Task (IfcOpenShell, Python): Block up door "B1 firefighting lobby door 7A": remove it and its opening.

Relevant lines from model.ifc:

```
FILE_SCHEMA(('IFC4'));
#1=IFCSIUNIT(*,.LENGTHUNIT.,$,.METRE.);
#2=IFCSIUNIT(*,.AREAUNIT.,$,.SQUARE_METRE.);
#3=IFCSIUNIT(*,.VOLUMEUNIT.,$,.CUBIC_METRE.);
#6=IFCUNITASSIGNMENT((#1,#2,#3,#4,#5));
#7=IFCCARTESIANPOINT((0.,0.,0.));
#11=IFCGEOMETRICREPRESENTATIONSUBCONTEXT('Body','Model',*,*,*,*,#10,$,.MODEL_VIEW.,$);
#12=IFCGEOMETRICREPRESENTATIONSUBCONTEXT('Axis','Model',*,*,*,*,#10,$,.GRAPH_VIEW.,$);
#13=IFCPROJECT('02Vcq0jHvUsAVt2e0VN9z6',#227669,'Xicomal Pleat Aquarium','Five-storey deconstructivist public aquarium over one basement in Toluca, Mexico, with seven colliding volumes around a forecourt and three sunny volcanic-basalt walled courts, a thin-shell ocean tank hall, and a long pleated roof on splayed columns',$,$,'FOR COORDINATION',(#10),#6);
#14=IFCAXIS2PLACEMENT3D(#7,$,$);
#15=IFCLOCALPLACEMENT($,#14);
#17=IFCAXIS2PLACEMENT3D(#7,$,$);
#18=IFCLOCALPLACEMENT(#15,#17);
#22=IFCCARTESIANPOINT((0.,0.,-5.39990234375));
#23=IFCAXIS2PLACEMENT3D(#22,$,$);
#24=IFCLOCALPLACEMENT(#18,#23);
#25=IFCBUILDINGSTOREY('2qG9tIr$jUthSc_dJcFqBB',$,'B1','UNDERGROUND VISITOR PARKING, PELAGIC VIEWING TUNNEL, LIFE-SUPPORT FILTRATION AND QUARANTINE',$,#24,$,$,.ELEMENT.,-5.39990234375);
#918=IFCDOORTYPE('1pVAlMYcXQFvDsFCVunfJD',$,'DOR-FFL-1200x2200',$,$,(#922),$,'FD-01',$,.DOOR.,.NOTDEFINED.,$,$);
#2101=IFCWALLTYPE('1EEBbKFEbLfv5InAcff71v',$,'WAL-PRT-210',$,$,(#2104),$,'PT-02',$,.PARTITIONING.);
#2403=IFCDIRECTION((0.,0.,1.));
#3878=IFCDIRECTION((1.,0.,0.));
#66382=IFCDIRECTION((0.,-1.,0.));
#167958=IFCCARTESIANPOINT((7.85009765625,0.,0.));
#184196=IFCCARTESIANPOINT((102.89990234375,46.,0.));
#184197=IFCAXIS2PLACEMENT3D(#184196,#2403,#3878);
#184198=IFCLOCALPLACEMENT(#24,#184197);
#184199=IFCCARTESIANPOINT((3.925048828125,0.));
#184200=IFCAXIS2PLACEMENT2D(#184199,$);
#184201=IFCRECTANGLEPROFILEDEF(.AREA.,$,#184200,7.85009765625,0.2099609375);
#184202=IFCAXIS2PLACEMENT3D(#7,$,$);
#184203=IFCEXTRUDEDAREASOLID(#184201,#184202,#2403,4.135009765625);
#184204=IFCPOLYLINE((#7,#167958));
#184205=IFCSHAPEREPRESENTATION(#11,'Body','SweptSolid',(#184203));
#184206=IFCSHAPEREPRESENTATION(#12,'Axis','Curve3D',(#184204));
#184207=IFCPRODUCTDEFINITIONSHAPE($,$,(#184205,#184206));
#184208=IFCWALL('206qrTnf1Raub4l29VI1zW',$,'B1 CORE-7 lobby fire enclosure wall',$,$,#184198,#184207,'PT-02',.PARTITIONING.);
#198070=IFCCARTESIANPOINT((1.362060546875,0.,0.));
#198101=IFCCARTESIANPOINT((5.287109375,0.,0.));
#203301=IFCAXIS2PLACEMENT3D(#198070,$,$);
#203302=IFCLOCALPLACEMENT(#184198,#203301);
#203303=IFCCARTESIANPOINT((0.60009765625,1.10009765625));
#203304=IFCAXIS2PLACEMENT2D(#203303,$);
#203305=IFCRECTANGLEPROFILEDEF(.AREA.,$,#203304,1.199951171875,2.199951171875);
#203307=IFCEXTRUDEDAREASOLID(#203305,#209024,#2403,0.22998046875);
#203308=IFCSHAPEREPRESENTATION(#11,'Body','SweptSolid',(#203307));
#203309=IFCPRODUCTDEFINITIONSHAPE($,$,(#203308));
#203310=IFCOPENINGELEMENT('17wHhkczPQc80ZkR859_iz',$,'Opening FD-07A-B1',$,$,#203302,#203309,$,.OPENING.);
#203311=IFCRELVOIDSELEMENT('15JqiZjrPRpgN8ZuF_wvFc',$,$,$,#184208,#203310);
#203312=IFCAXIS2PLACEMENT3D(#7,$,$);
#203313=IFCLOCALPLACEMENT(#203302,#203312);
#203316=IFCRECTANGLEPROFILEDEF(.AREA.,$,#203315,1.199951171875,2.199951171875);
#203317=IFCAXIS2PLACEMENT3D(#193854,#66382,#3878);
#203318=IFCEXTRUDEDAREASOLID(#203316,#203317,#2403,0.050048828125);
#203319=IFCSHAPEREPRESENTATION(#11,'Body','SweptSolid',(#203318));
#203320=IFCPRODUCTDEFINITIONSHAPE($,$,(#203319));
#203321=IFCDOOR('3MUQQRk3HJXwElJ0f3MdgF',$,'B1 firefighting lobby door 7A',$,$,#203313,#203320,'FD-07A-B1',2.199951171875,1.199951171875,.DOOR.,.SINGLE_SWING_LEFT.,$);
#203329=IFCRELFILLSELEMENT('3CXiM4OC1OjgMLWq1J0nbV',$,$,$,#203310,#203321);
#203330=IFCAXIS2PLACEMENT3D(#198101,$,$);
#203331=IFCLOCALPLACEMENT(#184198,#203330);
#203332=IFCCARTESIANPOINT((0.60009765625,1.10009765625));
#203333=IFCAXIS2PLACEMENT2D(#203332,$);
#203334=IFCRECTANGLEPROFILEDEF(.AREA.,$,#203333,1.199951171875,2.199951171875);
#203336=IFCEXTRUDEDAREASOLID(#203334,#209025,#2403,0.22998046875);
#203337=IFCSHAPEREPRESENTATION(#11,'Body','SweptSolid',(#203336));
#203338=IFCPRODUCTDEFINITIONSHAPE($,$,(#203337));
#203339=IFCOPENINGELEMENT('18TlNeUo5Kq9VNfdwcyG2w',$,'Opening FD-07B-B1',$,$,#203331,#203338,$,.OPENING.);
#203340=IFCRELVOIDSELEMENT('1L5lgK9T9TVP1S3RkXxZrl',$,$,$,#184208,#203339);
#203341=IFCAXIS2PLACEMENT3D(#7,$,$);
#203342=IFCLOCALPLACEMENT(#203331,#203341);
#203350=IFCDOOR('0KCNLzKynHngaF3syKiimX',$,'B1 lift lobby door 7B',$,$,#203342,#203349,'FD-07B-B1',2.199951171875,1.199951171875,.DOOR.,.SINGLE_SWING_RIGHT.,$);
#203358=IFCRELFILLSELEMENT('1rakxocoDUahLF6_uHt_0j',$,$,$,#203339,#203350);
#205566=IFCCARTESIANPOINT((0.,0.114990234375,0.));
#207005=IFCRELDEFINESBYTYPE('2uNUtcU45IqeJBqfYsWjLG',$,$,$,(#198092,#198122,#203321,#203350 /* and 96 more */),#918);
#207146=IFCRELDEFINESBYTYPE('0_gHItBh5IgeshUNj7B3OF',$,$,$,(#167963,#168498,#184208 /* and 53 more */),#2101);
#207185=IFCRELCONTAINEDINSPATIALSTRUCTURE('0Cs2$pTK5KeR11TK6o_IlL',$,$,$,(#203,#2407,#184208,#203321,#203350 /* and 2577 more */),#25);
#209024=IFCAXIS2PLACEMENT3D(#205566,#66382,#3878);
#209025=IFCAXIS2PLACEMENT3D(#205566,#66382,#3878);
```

```python
import ifcopenshell
import ifcopenshell.api.feature
import ifcopenshell.api.root
import ifcopenshell.geom
import ifcopenshell.util.shape

model = ifcopenshell.open("model.ifc")
settings = ifcopenshell.geom.settings()


def volume(element):
    """Net volume in cubic metres, openings subtracted."""
    shape = ifcopenshell.geom.create_shape(settings, element)
    return ifcopenshell.util.shape.get_volume(shape.geometry)


door = model.by_id(203321)
opening = door.FillsVoids[0].RelatingOpeningElement
wall = opening.VoidsElements[0].RelatingBuildingElement
before = volume(wall)

ifcopenshell.api.root.remove_product(model, product=door)
ifcopenshell.api.feature.remove_feature(model, feature=opening)

after = volume(wall)

print(f"wall volume {before:.3f} -> {after:.3f} m3")

model.write("model_edited.ifc")
```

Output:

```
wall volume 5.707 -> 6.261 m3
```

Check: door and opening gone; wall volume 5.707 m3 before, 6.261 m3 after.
